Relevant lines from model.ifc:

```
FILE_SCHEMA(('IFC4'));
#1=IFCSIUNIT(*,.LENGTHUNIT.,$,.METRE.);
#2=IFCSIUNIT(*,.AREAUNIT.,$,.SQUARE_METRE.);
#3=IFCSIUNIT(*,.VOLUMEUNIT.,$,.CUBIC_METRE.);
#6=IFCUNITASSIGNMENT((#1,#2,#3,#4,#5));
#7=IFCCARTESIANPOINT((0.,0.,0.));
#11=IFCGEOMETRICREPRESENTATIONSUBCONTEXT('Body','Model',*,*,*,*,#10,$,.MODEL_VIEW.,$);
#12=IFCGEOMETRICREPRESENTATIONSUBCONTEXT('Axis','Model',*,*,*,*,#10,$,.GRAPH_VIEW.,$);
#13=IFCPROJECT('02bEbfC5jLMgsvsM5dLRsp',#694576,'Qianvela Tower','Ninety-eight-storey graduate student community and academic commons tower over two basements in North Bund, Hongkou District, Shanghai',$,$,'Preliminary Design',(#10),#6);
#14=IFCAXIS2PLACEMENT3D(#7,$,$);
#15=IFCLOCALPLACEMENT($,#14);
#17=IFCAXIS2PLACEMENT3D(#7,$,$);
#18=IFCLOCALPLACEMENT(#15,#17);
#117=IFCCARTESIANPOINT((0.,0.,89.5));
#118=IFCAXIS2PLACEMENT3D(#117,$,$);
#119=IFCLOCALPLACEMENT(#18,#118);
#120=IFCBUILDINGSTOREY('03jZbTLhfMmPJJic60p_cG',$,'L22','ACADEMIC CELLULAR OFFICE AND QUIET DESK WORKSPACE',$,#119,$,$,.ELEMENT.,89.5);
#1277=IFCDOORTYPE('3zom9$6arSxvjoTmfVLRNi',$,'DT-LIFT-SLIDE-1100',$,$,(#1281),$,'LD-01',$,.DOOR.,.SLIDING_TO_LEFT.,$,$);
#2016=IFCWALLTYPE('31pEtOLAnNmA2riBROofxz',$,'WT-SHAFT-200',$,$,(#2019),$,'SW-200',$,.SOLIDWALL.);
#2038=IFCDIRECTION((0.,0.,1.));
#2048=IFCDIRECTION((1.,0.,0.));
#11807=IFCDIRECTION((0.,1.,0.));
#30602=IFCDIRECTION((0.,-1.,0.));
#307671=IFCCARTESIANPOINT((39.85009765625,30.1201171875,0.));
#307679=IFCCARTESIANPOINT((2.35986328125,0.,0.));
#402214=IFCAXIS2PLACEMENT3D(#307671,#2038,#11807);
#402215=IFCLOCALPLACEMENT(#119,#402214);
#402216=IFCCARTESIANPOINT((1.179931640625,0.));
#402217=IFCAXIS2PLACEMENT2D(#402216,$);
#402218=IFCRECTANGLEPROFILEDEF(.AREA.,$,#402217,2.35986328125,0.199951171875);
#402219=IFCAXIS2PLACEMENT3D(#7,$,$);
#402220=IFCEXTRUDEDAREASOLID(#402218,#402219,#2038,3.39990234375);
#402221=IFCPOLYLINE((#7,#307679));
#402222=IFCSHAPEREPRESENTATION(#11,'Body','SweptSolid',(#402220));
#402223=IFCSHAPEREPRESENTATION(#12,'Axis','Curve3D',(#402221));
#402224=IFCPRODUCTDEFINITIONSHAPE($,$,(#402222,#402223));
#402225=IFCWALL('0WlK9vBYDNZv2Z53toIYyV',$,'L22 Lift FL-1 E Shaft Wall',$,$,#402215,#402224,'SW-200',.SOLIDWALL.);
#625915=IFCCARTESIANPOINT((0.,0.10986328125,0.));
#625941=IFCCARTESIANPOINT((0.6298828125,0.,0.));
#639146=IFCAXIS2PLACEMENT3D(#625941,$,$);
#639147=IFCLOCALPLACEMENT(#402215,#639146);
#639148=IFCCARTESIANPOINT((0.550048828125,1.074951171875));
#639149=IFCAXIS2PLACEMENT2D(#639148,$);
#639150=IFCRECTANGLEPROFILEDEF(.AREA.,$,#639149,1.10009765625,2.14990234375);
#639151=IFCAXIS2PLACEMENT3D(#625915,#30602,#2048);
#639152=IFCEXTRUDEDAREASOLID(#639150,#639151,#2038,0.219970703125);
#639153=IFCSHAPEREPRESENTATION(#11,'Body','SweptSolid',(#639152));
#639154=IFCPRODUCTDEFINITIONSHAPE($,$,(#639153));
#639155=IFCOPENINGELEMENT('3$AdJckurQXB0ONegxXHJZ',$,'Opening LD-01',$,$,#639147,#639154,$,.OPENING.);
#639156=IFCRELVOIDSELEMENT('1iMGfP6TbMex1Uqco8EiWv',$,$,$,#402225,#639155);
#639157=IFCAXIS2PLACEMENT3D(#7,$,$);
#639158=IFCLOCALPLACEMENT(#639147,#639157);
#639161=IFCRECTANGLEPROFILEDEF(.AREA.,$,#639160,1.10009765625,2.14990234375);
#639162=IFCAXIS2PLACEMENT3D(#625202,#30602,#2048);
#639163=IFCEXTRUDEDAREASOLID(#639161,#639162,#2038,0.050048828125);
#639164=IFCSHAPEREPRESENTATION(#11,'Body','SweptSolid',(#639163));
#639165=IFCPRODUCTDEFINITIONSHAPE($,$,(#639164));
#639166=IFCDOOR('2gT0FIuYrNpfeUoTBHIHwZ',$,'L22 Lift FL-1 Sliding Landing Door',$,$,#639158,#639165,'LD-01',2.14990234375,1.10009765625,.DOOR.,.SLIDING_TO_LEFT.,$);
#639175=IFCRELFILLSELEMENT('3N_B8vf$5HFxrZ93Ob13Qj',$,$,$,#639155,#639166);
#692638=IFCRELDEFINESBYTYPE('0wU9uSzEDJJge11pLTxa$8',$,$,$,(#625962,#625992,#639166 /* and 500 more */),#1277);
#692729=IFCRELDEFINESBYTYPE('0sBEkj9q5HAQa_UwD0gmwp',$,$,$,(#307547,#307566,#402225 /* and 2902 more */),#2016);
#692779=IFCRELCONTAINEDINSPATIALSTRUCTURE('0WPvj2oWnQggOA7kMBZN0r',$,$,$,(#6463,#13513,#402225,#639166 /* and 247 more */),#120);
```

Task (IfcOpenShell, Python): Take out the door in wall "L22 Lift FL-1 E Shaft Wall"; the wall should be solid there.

```python
import ifcopenshell
import ifcopenshell.api.feature
import ifcopenshell.api.root
import ifcopenshell.geom
import ifcopenshell.util.shape

model = ifcopenshell.open("model.ifc")
settings = ifcopenshell.geom.settings()


def volume(element):
    """Net volume in cubic metres, openings subtracted."""
    shape = ifcopenshell.geom.create_shape(settings, element)
    return ifcopenshell.util.shape.get_volume(shape.geometry)


door = model.by_guid("2gT0FIuYrNpfeUoTBHIHwZ")
opening = door.FillsVoids[0].RelatingOpeningElement
wall = opening.VoidsElements[0].RelatingBuildingElement
before = volume(wall)

ifcopenshell.api.root.remove_product(model, product=door)
ifcopenshell.api.feature.remove_feature(model, feature=opening)

after = volume(wall)

print(f"wall volume {before:.3f} -> {after:.3f} m3")

model.write("model_v2.ifc")
```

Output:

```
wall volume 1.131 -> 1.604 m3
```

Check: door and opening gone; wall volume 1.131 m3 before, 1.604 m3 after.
